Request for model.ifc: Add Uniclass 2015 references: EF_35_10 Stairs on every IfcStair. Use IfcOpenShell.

First a look at what the model holds.

```python
import ifcopenshell

model = ifcopenshell.open("model.ifc")
print(model.schema)
print("classifications:", [c.Name for c in model.by_type("IfcClassification")])
for ifc_class in ("IfcDoor", "IfcRoof", "IfcStair", "IfcWall", "IfcWindow"):
    print(ifc_class, len(model.by_type(ifc_class)))
```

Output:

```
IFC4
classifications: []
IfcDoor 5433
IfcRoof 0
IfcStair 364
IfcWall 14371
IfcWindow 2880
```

```python
import ifcopenshell
import ifcopenshell.api.classification

model = ifcopenshell.open("model.ifc")

system = ifcopenshell.api.classification.add_classification(model, classification="Uniclass 2015")

codes = {
    "IfcStair": ("EF_35_10", "Stairs"),
}
for ifc_class, (code, name) in codes.items():
    products = model.by_type(ifc_class)
    ifcopenshell.api.classification.add_reference(
        model, products=products, classification=system, identification=code, name=name
    )
    print(code, len(products))

model.write("model_rev.ifc")
```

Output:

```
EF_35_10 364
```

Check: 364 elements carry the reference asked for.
